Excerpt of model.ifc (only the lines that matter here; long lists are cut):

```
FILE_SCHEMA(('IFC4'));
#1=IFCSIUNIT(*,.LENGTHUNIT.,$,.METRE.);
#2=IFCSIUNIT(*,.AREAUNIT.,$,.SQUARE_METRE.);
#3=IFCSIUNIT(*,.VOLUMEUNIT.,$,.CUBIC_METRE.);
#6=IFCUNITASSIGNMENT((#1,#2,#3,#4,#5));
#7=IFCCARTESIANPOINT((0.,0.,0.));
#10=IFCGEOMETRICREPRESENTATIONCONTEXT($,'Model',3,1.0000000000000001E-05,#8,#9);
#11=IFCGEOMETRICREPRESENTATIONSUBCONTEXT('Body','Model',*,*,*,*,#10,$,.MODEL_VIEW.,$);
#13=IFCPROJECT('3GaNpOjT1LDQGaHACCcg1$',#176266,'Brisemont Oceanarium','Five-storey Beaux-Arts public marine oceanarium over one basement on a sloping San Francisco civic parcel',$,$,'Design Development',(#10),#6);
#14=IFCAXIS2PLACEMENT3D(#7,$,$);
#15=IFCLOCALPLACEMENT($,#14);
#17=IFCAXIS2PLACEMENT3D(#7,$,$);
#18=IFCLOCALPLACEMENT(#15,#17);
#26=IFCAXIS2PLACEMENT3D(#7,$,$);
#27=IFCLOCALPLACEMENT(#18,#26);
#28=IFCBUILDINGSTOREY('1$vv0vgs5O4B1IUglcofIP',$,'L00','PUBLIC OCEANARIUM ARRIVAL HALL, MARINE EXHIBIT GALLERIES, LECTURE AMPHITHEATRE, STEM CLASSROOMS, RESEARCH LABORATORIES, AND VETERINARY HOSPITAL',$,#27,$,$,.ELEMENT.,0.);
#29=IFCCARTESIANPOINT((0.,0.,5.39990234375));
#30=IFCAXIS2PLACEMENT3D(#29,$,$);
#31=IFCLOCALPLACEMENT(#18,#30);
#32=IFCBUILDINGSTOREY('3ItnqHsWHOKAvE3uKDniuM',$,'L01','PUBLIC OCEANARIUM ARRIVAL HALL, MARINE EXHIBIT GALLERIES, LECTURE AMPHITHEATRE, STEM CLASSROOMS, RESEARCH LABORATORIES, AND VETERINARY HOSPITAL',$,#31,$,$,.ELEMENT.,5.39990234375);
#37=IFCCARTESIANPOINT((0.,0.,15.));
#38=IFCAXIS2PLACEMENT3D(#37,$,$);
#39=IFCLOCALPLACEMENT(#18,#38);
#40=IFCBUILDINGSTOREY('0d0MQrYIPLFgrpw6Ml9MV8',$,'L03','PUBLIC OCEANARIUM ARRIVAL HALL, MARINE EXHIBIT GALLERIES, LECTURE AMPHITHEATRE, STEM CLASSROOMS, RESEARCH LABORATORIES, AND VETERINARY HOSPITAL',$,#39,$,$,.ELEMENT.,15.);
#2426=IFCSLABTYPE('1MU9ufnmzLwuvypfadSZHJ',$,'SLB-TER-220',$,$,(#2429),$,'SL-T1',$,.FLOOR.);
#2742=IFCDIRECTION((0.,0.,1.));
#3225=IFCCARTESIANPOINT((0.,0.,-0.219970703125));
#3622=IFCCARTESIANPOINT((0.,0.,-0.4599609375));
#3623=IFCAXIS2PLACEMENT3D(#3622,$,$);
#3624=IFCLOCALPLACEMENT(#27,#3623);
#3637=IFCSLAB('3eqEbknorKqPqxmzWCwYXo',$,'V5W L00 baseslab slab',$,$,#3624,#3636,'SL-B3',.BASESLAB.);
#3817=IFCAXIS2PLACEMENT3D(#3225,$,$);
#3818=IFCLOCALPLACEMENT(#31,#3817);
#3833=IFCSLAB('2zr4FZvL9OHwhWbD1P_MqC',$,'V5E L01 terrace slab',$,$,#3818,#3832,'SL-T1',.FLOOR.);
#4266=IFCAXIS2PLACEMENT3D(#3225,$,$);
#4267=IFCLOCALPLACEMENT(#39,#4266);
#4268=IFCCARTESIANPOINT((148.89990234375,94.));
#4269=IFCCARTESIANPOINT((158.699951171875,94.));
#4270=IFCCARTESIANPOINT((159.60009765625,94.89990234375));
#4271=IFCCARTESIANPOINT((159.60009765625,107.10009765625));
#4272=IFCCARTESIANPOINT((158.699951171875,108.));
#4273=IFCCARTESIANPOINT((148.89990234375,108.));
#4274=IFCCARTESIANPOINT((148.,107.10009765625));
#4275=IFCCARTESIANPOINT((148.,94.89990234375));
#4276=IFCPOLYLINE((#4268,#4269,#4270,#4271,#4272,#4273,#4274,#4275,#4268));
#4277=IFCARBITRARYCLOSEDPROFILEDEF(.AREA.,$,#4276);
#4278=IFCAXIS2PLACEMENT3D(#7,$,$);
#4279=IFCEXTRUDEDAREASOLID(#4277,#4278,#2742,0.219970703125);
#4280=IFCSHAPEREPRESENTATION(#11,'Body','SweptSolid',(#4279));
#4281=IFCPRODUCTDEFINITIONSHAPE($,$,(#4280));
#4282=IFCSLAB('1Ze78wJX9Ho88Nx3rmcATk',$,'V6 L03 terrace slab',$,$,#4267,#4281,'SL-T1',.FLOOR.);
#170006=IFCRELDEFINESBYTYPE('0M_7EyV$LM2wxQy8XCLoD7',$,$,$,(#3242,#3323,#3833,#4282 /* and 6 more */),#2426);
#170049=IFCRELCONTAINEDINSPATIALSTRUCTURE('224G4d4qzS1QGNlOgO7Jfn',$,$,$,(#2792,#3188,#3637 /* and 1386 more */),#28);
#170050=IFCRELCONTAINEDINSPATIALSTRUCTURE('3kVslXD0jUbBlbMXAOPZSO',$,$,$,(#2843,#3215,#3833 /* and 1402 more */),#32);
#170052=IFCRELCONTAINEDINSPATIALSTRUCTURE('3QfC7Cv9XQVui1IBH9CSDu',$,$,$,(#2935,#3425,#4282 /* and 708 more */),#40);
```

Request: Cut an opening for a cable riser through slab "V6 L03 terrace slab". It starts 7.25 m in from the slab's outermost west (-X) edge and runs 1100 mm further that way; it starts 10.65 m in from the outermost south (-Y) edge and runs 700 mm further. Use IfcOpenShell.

```python
import numpy as np
import ifcopenshell
import ifcopenshell.api.feature
import ifcopenshell.api.geometry
import ifcopenshell.api.root
import ifcopenshell.geom
import ifcopenshell.util.placement
import ifcopenshell.util.representation
import ifcopenshell.util.shape
import ifcopenshell.util.unit

model = ifcopenshell.open("model.ifc")
unit_scale = ifcopenshell.util.unit.calculate_unit_scale(model)
settings = ifcopenshell.geom.settings()


def volume(element):
    """Net volume in cubic metres, openings subtracted."""
    shape = ifcopenshell.geom.create_shape(settings, element)
    return ifcopenshell.util.shape.get_volume(shape.geometry)


slab = model.by_guid("1Ze78wJX9Ho88Nx3rmcATk")
before = volume(slab)

# Extent in the slab's own axes, in metres. The edges named are its -X and -Y sides.
slab_shape = ifcopenshell.geom.create_shape(settings, slab)
vertices = ifcopenshell.util.shape.get_vertices(slab_shape.geometry)
x_min, y_min, bottom = vertices.min(axis=0)
top = vertices[:, 2].max()

opening = ifcopenshell.api.root.create_entity(model, ifc_class="IfcOpeningElement", name="Cable riser opening", predefined_type="OPENING")
context = ifcopenshell.util.representation.get_context(model, "Model", "Body", "MODEL_VIEW")
width, depth = 1.1, 0.7
outline = [(0.0, 0.0), (width, 0.0), (width, depth), (0.0, depth), (0.0, 0.0)]
# Overshoot both faces by 50 mm so the cut is clean.
shape = ifcopenshell.api.geometry.add_slab_representation(
    model, context=context, depth=top - bottom + 0.1, polyline=outline
)
ifcopenshell.api.geometry.assign_representation(model, product=opening, representation=shape)

matrix = ifcopenshell.util.placement.get_local_placement(slab.ObjectPlacement)
matrix[:, 3] = matrix @ np.append(np.array([x_min + 7.25, y_min + 10.65, bottom - 0.05]) / unit_scale, 1.0)
ifcopenshell.api.geometry.edit_object_placement(model, product=opening, matrix=matrix, is_si=False)
ifcopenshell.api.feature.add_feature(model, feature=opening, element=slab)

after = volume(slab)

print(f"slab volume {before:.3f} -> {after:.3f} m3")

model.write("model_rev.ifc")
```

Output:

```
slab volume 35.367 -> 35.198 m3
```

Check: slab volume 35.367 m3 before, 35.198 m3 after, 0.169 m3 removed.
